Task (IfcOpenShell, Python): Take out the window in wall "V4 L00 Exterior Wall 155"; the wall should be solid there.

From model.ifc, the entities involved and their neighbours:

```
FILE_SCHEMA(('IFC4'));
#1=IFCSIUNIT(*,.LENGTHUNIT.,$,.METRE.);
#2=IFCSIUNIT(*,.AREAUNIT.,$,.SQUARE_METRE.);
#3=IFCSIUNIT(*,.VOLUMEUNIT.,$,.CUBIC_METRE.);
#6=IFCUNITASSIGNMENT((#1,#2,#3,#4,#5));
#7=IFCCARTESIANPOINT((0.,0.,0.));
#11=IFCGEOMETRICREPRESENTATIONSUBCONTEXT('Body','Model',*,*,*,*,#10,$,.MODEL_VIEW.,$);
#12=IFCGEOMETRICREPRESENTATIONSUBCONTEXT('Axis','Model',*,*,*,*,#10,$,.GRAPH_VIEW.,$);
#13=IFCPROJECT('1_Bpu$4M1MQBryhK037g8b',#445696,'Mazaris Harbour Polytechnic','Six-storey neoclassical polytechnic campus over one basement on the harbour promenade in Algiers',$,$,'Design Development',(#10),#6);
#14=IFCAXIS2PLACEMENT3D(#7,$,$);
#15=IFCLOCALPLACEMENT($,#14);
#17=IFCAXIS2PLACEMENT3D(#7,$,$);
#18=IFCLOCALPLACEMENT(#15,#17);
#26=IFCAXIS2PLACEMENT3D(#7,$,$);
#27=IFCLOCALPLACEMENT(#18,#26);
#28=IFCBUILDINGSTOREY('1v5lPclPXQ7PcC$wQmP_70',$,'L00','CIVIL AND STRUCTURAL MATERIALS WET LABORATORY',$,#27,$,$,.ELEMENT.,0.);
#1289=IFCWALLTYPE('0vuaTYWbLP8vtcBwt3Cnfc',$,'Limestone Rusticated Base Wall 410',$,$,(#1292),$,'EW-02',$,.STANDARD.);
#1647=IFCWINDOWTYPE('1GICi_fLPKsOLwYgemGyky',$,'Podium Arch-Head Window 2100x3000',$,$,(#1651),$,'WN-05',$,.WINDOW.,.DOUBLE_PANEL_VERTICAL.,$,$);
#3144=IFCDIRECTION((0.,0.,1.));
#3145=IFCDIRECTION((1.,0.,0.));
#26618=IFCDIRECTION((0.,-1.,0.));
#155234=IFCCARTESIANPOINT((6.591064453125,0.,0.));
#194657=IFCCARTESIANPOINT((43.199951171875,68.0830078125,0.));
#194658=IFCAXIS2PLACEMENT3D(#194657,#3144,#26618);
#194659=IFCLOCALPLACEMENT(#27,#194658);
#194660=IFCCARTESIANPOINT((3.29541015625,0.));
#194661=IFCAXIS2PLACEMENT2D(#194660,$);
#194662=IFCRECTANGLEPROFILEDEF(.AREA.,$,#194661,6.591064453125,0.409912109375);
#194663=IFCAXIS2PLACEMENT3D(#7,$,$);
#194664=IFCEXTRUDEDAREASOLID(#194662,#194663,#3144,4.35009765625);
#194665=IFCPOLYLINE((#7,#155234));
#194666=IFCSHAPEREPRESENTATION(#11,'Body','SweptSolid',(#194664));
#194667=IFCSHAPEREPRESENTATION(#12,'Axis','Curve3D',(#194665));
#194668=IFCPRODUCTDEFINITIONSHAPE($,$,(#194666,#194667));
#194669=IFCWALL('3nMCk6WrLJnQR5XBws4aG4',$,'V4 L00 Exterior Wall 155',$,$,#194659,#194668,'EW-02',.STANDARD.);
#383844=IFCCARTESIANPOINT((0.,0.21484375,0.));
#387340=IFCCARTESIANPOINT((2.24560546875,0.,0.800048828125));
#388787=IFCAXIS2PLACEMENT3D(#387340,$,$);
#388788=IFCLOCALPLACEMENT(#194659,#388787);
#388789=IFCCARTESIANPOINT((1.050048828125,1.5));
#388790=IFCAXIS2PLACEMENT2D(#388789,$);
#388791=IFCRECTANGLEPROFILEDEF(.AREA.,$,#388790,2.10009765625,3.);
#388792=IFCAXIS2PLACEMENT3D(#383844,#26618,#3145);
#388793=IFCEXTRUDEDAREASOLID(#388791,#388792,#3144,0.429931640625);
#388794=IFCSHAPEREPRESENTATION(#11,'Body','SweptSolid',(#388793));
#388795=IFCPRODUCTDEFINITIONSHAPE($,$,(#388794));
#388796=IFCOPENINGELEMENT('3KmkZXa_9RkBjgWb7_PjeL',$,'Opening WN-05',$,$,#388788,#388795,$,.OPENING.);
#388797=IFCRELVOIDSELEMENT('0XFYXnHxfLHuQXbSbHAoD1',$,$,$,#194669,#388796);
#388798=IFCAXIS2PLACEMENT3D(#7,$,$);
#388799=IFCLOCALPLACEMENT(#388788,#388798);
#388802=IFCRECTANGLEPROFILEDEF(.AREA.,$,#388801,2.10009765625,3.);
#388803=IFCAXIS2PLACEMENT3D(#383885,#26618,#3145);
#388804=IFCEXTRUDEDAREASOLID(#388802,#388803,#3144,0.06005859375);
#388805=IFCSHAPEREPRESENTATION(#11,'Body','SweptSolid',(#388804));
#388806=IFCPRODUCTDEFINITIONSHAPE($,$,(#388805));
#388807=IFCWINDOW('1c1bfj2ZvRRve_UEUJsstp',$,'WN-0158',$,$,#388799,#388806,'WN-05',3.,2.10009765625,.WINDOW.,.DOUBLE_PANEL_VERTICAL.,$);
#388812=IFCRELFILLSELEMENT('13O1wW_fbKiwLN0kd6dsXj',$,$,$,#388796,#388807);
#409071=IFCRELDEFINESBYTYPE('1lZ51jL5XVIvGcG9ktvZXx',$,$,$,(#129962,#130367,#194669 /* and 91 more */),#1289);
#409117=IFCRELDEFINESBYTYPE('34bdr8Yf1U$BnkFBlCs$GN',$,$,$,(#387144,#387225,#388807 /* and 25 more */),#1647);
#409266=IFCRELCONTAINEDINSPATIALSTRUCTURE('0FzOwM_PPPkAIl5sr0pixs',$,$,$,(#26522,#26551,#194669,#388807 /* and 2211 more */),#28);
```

```python
import ifcopenshell
import ifcopenshell.api.feature
import ifcopenshell.api.root
import ifcopenshell.geom
import ifcopenshell.util.shape

model = ifcopenshell.open("model.ifc")
settings = ifcopenshell.geom.settings()


def volume(element):
    """Net volume in cubic metres, openings subtracted."""
    shape = ifcopenshell.geom.create_shape(settings, element)
    return ifcopenshell.util.shape.get_volume(shape.geometry)


window = model.by_guid("1c1bfj2ZvRRve_UEUJsstp")
opening = window.FillsVoids[0].RelatingOpeningElement
wall = opening.VoidsElements[0].RelatingBuildingElement
before = volume(wall)

ifcopenshell.api.root.remove_product(model, product=window)
ifcopenshell.api.feature.remove_feature(model, feature=opening)

after = volume(wall)

print(f"wall volume {before:.3f} -> {after:.3f} m3")

model.write("model_v2.ifc")
```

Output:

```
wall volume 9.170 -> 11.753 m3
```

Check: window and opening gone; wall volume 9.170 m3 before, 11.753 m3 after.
